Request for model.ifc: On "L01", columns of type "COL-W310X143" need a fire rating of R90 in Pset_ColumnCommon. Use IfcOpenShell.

First a look at what the model holds.

```python
import ifcopenshell
import ifcopenshell.util.element

model = ifcopenshell.open("model.ifc")
print(model.schema)
storey = next(s for s in model.by_type("IfcBuildingStorey") if s.Name == "L01")
columns = [e for e in ifcopenshell.util.element.get_decomposition(storey) if e.is_a("IfcColumn")]
seen = {}
for e in columns:
    element_type = ifcopenshell.util.element.get_type(e)
    key = (element_type.Name if element_type != e and element_type else None, ifcopenshell.util.element.get_pset(e, "Pset_ColumnCommon", "FireRating"))
    seen[key] = seen.get(key, 0) + 1
for (name, value), count in sorted(seen.items(), key=str):
    print(count, "x", name, "|", value)
```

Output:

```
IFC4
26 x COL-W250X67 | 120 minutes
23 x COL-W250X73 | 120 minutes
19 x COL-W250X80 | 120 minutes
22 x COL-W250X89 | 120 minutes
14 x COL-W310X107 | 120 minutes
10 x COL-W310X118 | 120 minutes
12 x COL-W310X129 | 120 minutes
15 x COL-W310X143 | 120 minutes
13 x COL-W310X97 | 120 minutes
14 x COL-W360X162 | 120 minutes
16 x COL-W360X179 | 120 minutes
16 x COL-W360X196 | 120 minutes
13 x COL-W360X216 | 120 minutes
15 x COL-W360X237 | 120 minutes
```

```python
import ifcopenshell
import ifcopenshell.api.pset
import ifcopenshell.util.element

model = ifcopenshell.open("model.ifc")

storey = next(s for s in model.by_type("IfcBuildingStorey") if s.Name == "L01")
columns = [e for e in ifcopenshell.util.element.get_decomposition(storey) if e.is_a("IfcColumn")]

count = 0
for e in columns:
    element_type = ifcopenshell.util.element.get_type(e)
    if element_type in (None, e) or element_type.Name != "COL-W310X143":
        continue
    # add_pset returns the element's existing set when there is one.
    pset = ifcopenshell.api.pset.add_pset(model, product=e, name="Pset_ColumnCommon")
    ifcopenshell.api.pset.edit_pset(model, pset=pset, properties={"FireRating": "R90"})
    count += 1

print(count, "columns updated")

model.write("model-out.ifc")
```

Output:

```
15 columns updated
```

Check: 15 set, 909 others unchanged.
